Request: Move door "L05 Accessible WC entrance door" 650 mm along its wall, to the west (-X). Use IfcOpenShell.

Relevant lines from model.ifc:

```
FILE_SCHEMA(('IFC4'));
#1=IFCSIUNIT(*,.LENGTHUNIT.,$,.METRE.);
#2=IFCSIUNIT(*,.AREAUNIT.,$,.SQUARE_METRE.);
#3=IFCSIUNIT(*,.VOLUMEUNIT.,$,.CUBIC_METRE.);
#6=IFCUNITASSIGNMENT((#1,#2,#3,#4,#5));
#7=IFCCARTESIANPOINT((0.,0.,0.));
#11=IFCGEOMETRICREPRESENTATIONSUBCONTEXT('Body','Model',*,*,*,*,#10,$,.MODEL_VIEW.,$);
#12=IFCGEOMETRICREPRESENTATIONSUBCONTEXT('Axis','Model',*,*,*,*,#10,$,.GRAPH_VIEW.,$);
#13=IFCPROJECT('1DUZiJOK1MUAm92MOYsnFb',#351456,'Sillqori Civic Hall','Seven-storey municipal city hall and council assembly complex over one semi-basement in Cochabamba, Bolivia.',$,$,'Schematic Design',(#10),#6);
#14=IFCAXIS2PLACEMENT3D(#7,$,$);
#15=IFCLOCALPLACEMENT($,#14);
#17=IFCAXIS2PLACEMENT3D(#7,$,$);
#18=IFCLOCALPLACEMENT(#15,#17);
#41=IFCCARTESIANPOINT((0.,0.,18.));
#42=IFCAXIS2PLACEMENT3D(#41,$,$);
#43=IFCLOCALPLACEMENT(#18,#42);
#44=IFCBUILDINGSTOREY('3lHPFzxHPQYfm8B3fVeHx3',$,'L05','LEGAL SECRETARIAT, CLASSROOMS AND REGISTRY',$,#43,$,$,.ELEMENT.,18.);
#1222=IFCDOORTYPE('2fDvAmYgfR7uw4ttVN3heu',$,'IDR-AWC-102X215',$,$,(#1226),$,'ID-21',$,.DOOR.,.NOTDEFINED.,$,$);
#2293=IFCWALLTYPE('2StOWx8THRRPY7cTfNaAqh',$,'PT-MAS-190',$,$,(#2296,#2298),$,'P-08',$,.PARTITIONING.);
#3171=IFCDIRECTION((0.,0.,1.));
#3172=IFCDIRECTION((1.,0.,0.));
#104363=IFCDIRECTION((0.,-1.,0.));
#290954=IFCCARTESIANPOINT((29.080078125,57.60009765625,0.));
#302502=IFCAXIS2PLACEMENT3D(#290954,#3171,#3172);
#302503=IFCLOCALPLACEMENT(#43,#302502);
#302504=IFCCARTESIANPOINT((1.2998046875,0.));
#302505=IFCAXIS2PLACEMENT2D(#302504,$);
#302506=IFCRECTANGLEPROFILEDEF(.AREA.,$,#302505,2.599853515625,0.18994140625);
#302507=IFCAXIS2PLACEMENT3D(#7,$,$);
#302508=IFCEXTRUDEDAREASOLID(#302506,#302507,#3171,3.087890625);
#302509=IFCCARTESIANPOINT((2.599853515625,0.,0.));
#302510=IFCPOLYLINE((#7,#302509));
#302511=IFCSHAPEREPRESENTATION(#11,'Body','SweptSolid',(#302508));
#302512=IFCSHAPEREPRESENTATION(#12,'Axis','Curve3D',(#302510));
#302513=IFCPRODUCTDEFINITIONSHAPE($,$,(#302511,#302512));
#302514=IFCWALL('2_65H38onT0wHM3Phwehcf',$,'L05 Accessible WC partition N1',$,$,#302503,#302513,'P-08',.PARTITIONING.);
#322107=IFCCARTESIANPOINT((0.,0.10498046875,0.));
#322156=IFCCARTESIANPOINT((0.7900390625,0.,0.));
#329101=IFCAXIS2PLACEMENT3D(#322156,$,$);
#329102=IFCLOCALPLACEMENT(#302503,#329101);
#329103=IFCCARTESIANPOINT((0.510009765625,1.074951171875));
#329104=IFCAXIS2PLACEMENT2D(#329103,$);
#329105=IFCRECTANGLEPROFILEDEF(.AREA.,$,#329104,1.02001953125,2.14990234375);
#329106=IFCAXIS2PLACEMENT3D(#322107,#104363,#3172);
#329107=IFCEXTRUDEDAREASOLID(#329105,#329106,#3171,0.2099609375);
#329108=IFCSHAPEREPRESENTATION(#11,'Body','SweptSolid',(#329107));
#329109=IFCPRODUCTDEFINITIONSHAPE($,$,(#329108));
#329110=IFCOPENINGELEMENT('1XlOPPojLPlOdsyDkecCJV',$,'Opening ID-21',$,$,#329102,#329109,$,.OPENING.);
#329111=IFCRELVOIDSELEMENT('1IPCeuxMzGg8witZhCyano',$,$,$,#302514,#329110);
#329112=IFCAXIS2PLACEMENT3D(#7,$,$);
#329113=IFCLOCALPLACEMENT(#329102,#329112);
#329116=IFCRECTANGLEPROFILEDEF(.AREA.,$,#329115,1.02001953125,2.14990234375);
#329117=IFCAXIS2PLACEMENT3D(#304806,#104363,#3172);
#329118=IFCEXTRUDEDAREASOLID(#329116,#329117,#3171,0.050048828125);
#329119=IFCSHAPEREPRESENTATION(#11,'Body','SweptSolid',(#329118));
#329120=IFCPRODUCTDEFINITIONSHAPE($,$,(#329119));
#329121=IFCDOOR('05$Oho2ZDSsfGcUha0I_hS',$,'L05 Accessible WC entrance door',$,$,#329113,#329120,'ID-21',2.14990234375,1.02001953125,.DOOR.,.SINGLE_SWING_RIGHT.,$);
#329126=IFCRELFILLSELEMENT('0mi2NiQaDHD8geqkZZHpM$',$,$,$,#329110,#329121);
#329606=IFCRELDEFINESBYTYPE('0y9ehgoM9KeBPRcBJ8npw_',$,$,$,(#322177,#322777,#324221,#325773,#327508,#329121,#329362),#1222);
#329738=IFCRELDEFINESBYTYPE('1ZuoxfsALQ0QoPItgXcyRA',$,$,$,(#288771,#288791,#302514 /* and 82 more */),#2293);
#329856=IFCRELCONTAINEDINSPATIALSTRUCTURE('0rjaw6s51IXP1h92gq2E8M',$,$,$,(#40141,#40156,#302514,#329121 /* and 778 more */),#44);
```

```python
import ifcopenshell
import ifcopenshell.api.geometry
import ifcopenshell.util.placement

model = ifcopenshell.open("model.ifc")

door = model.by_guid("05$Oho2ZDSsfGcUha0I_hS")
opening = door.FillsVoids[0].RelatingOpeningElement
wall = opening.VoidsElements[0].RelatingBuildingElement

wall_matrix = ifcopenshell.util.placement.get_local_placement(wall.ObjectPlacement)
shift = wall_matrix[:3, 0] * -0.65
before = ifcopenshell.util.placement.get_local_placement(door.ObjectPlacement)[:3, 3].copy()

# The door is placed relative to its opening, so it follows when the opening moves.
matrix = ifcopenshell.util.placement.get_local_placement(opening.ObjectPlacement)
matrix[:3, 3] += shift
ifcopenshell.api.geometry.edit_object_placement(
    model, product=opening, matrix=matrix, is_si=False, should_transform_children=True
)

after = ifcopenshell.util.placement.get_local_placement(door.ObjectPlacement)[:3, 3]
print("door moved by", (after - before).round(3) + 0.0)

model.write("model-out.ifc")
```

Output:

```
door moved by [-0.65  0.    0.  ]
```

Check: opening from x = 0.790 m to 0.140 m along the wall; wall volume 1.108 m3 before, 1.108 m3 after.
